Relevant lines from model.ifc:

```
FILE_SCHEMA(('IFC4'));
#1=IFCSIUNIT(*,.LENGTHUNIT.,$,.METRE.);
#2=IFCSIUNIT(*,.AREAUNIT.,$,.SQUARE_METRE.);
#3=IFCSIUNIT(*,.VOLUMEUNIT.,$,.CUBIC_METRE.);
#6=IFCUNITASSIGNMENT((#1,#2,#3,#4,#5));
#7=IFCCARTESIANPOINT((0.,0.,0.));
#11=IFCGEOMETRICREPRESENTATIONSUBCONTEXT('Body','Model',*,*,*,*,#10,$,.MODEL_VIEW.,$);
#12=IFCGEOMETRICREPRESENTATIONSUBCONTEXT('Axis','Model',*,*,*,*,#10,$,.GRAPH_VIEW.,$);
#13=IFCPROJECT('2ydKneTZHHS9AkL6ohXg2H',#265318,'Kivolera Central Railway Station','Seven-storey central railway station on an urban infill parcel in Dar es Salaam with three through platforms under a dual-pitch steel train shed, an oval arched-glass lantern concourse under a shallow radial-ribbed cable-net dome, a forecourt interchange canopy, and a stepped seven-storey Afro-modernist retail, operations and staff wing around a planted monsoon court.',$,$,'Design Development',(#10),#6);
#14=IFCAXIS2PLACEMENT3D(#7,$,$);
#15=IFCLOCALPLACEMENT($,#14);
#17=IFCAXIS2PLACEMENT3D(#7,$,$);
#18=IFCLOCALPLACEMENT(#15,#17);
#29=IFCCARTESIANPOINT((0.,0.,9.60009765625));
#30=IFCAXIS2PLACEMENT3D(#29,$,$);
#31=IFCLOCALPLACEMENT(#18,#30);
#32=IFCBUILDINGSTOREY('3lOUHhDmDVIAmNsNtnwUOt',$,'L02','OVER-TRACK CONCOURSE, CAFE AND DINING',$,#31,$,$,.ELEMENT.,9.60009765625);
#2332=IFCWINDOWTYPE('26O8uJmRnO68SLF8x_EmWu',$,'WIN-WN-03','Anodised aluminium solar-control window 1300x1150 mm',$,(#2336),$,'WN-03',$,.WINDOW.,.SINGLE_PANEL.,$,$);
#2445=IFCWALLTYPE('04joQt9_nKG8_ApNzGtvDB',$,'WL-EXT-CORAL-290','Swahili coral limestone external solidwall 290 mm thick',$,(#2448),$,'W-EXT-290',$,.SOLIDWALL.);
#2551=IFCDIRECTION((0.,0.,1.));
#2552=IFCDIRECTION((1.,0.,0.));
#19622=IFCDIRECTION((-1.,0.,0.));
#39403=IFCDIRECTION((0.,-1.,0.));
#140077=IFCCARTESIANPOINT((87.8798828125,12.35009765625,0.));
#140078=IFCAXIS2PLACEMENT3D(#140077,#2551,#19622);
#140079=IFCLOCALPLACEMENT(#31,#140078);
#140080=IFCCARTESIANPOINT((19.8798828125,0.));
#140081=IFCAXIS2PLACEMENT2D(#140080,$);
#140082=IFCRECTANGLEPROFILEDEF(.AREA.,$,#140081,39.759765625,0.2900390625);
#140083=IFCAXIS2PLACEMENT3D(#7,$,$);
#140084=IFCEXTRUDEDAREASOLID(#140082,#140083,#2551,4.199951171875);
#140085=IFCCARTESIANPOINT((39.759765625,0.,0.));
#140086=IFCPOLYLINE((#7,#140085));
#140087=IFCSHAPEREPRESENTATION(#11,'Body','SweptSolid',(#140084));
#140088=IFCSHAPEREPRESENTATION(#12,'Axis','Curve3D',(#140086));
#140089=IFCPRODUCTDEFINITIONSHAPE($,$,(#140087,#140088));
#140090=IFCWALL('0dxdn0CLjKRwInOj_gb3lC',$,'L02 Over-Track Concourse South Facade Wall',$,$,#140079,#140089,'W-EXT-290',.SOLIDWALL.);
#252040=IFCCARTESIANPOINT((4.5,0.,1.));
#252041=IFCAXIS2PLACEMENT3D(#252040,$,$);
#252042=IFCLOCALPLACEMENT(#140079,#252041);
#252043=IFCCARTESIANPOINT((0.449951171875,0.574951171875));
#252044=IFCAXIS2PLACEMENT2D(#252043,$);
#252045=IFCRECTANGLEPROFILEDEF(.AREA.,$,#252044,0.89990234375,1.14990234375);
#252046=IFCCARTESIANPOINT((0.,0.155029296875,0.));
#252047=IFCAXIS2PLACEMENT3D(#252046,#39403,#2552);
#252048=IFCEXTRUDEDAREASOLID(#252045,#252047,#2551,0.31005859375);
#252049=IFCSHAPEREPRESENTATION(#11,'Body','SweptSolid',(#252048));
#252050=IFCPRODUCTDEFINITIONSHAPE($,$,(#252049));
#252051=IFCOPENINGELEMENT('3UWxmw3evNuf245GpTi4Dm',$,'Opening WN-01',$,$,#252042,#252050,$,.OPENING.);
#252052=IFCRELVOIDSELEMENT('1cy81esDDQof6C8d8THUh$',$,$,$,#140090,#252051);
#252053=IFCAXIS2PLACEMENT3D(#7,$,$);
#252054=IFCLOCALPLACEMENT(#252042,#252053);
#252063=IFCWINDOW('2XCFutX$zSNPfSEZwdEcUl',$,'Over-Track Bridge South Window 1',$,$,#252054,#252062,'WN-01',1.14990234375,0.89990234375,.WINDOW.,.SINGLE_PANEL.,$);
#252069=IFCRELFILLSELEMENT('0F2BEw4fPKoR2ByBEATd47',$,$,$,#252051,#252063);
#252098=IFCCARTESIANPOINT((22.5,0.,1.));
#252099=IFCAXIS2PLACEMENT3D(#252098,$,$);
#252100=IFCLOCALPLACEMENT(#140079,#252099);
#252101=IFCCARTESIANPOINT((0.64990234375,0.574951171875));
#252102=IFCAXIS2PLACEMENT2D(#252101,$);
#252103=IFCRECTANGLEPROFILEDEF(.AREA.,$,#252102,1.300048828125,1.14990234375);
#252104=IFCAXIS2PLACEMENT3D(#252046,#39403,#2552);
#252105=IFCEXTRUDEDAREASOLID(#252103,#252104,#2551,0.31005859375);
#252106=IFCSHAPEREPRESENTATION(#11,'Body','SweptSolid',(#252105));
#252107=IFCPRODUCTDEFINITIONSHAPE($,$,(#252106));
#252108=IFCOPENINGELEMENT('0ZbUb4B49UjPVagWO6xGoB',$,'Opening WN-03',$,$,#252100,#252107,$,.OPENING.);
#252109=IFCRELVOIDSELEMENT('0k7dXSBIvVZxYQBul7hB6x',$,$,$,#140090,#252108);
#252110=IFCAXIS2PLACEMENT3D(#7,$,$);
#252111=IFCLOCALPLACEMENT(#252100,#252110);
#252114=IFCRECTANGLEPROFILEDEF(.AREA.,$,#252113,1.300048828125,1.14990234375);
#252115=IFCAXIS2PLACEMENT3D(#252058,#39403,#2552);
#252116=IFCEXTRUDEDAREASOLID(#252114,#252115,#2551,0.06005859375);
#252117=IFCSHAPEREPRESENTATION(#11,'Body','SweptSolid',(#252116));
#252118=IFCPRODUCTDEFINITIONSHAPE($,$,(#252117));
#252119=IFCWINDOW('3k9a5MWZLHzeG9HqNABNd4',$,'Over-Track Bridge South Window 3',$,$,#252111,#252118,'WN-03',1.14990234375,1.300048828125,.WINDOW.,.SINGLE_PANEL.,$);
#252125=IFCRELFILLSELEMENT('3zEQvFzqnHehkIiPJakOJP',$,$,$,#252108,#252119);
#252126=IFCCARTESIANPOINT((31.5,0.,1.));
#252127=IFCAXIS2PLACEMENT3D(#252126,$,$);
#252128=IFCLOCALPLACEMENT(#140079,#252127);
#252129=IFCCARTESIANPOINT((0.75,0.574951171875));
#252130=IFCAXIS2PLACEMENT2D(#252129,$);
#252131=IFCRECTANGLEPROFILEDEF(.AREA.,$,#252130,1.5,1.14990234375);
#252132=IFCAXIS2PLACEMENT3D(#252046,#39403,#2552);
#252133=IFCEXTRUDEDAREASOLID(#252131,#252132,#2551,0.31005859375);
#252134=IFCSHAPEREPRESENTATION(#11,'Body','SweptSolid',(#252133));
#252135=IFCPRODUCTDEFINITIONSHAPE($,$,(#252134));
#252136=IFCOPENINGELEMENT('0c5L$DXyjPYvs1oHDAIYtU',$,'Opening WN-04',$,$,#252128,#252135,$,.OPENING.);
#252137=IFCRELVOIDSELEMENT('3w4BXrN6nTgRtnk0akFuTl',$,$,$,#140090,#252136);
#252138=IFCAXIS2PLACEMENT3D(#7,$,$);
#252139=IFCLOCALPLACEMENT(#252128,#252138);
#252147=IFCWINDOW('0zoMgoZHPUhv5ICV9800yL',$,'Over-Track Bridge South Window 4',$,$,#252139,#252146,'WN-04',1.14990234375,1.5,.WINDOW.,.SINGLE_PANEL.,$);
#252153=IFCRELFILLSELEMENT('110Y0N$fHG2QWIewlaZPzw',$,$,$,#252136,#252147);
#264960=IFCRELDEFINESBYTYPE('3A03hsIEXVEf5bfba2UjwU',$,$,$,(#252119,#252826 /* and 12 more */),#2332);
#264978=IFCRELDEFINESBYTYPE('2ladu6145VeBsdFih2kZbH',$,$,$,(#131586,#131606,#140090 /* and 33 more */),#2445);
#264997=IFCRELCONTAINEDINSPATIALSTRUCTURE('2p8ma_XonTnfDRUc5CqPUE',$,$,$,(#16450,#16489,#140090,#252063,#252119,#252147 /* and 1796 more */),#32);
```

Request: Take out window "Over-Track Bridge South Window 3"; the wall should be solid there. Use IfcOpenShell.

```python
import ifcopenshell
import ifcopenshell.api.feature
import ifcopenshell.api.root
import ifcopenshell.geom
import ifcopenshell.util.shape

model = ifcopenshell.open("model.ifc")
settings = ifcopenshell.geom.settings()


def volume(element):
    """Net volume in cubic metres, openings subtracted."""
    shape = ifcopenshell.geom.create_shape(settings, element)
    return ifcopenshell.util.shape.get_volume(shape.geometry)


window = model.by_guid("3k9a5MWZLHzeG9HqNABNd4")
opening = window.FillsVoids[0].RelatingOpeningElement
wall = opening.VoidsElements[0].RelatingBuildingElement
before = volume(wall)

ifcopenshell.api.root.remove_product(model, product=window)
ifcopenshell.api.feature.remove_feature(model, feature=opening)

after = volume(wall)

print(f"wall volume {before:.3f} -> {after:.3f} m3")

model.write("model_v2.ifc")
```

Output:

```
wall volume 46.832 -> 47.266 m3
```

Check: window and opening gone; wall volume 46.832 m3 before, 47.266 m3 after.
